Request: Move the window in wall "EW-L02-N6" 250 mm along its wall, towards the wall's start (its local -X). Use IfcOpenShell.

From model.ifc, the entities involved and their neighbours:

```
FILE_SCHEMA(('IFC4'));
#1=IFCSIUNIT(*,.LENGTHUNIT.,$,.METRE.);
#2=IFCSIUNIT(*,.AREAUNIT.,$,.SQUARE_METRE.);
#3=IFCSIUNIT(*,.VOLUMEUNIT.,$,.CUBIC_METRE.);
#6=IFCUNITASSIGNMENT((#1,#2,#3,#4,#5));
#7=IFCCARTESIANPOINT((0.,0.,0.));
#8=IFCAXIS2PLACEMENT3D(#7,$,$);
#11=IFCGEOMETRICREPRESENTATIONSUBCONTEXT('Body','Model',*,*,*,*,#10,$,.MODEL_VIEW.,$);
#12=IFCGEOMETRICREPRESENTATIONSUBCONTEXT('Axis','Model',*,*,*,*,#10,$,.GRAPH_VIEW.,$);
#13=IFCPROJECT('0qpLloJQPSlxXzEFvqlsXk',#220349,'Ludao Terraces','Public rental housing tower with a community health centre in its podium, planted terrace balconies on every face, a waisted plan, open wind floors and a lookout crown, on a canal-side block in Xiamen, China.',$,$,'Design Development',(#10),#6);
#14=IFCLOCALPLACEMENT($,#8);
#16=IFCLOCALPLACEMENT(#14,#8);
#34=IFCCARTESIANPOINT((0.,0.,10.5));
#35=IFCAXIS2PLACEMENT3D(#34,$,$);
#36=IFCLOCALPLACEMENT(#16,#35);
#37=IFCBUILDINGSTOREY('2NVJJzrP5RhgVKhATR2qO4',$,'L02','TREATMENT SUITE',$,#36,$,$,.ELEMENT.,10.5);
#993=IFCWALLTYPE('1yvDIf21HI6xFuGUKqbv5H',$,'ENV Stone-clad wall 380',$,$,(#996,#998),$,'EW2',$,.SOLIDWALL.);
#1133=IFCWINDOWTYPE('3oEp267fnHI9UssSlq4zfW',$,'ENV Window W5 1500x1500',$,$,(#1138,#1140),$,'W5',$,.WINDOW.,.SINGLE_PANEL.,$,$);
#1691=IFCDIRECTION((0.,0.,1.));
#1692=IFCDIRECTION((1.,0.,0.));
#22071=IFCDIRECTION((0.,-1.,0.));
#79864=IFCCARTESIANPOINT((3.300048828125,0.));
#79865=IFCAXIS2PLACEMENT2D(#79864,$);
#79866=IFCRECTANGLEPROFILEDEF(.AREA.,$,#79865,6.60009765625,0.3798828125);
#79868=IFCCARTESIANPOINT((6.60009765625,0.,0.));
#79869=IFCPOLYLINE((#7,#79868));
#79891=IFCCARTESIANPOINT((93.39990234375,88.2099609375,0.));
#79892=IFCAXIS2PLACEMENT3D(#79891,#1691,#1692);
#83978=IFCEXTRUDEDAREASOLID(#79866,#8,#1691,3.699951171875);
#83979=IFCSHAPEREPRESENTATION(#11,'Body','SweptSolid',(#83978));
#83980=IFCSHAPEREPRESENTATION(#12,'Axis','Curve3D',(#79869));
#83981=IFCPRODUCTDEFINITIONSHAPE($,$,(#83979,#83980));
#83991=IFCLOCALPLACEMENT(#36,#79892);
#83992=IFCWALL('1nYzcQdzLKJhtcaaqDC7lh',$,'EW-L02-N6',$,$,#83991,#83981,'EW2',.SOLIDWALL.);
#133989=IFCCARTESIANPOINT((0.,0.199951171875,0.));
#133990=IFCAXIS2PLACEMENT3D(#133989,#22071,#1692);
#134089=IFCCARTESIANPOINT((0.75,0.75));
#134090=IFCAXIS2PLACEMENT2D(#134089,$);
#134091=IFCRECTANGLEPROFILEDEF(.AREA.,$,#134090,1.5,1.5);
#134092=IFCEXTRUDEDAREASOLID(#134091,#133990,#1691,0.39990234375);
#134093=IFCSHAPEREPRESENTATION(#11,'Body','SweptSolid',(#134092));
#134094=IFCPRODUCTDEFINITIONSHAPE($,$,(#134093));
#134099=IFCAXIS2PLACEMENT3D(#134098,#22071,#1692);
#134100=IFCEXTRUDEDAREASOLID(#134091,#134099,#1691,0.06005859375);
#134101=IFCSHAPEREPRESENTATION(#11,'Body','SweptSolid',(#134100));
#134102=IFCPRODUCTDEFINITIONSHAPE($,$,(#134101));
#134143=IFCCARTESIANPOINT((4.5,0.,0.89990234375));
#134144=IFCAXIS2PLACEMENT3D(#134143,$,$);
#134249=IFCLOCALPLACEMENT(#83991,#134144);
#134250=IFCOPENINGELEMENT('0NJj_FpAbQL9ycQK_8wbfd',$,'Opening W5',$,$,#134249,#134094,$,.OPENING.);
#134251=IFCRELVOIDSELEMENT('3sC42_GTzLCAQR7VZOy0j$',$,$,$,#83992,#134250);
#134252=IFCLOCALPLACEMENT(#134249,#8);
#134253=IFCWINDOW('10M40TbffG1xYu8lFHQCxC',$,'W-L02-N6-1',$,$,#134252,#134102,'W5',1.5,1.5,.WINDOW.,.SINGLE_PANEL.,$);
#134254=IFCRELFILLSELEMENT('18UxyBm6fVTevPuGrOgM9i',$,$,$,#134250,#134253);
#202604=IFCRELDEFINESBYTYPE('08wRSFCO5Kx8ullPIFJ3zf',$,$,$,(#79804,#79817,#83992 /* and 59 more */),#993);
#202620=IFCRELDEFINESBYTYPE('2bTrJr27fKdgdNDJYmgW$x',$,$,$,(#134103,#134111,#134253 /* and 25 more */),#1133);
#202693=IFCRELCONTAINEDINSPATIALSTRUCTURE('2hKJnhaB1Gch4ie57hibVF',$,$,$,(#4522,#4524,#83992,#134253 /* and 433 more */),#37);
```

```python
import ifcopenshell
import ifcopenshell.api.geometry
import ifcopenshell.util.placement

model = ifcopenshell.open("model.ifc")

window = model.by_guid("10M40TbffG1xYu8lFHQCxC")
opening = window.FillsVoids[0].RelatingOpeningElement
wall = opening.VoidsElements[0].RelatingBuildingElement

wall_matrix = ifcopenshell.util.placement.get_local_placement(wall.ObjectPlacement)
shift = wall_matrix[:3, 0] * -0.25
before = ifcopenshell.util.placement.get_local_placement(window.ObjectPlacement)[:3, 3].copy()

# The window is placed relative to its opening, so it follows when the opening moves.
matrix = ifcopenshell.util.placement.get_local_placement(opening.ObjectPlacement)
matrix[:3, 3] += shift
ifcopenshell.api.geometry.edit_object_placement(
    model, product=opening, matrix=matrix, is_si=False, should_transform_children=True
)

after = ifcopenshell.util.placement.get_local_placement(window.ObjectPlacement)[:3, 3]
print("window moved by", (after - before).round(3) + 0.0)

model.write("model_edited.ifc")
```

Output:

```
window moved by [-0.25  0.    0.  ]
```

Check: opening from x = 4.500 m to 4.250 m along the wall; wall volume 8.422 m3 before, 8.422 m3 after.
